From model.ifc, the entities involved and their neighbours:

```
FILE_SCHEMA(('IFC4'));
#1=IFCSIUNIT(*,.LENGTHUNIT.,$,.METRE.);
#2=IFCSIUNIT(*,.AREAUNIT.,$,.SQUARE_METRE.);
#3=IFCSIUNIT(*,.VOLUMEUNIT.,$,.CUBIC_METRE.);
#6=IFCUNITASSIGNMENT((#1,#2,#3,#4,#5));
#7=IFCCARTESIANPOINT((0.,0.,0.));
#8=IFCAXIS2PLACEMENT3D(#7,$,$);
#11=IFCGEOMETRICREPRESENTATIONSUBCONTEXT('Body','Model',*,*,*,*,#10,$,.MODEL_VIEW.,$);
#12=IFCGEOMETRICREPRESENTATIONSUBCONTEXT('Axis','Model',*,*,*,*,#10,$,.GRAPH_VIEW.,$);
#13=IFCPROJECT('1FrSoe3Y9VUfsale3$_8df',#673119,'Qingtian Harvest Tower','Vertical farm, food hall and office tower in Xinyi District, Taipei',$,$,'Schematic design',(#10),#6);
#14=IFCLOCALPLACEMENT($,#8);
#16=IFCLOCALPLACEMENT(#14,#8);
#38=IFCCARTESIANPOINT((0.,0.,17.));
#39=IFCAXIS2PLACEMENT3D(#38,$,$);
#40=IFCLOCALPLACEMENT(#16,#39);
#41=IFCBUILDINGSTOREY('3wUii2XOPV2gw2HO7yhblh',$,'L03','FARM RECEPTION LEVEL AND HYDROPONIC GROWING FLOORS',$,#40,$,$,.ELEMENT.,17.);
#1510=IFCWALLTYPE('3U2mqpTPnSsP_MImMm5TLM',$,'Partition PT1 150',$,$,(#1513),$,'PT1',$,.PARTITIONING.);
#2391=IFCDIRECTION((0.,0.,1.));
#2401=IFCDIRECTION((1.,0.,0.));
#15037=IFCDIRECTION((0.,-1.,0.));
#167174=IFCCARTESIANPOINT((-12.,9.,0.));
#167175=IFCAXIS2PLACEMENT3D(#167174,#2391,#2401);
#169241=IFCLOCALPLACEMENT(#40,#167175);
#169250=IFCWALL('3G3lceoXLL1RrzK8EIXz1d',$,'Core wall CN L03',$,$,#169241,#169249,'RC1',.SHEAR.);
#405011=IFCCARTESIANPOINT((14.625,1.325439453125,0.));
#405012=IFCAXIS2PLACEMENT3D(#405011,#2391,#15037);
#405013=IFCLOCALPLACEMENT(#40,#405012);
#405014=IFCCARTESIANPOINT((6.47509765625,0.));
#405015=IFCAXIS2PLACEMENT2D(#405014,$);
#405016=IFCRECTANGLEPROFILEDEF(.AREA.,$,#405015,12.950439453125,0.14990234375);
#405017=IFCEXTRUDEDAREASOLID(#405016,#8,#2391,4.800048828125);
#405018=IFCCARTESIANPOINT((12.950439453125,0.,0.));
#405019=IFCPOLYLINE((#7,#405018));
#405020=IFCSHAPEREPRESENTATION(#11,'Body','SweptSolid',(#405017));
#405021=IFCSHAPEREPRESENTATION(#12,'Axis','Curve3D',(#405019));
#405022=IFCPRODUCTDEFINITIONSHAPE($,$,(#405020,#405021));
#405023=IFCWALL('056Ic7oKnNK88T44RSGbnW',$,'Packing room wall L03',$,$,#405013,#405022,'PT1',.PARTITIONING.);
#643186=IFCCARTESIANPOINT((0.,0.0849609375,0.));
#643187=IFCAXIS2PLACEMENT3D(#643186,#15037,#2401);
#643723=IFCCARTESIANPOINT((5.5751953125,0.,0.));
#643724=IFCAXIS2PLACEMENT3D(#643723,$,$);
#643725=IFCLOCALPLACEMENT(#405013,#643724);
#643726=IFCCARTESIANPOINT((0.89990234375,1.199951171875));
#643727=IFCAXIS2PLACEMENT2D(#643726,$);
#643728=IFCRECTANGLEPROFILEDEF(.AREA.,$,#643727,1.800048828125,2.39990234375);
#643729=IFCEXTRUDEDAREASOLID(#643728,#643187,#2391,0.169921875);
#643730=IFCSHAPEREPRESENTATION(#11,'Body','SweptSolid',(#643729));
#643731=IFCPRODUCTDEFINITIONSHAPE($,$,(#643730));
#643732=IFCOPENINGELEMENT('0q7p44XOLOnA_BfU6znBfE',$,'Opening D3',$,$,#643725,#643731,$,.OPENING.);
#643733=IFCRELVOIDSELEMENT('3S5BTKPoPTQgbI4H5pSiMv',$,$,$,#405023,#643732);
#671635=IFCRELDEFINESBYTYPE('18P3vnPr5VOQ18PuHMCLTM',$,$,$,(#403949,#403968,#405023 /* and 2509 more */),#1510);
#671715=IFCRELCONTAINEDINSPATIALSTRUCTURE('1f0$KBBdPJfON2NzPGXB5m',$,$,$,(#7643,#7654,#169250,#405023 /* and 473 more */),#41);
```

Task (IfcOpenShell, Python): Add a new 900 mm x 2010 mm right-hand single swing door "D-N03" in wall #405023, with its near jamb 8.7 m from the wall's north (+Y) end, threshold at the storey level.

```python
import numpy as np
import ifcopenshell
import ifcopenshell.api.feature
import ifcopenshell.api.geometry
import ifcopenshell.api.root
import ifcopenshell.api.spatial
import ifcopenshell.geom
import ifcopenshell.util.element
import ifcopenshell.util.placement
import ifcopenshell.util.representation
import ifcopenshell.util.shape
import ifcopenshell.util.unit

model = ifcopenshell.open("model.ifc")
unit_scale = ifcopenshell.util.unit.calculate_unit_scale(model)
settings = ifcopenshell.geom.settings()


def volume(element):
    """Net volume in cubic metres, openings subtracted."""
    shape = ifcopenshell.geom.create_shape(settings, element)
    return ifcopenshell.util.shape.get_volume(shape.geometry)


wall = model.by_id(405023)
storey = ifcopenshell.util.element.get_container(wall, ifc_class="IfcBuildingStorey")
context = ifcopenshell.util.representation.get_context(model, "Model", "Body", "MODEL_VIEW")
before = volume(wall)

width, height, from_end, sill = 0.9, 2.01, 8.7, 0.0  # metres

# The wall runs along its own X axis, and the end named is its -X end.
wall_shape = ifcopenshell.geom.create_shape(settings, wall)
x, y, z = ifcopenshell.util.shape.get_vertices(wall_shape.geometry).T
start = x.min() + from_end
face, thickness = float(y.min()), float(y.max() - y.min())
wall_matrix = ifcopenshell.util.placement.get_local_placement(wall.ObjectPlacement)
level = ifcopenshell.util.placement.get_local_placement(storey.ObjectPlacement)[2, 3]


def in_wall(x, y):
    """Placement at x, y metres in the wall's axes, at sill height."""
    matrix = wall_matrix.copy()
    matrix[:, 3] = wall_matrix @ np.array([x / unit_scale, y / unit_scale, 0.0, 1.0])
    matrix[2, 3] = level + sill / unit_scale
    return matrix


# Opening: a box that overshoots both wall faces by 50 mm.
opening = ifcopenshell.api.root.create_entity(model, ifc_class="IfcOpeningElement", predefined_type="OPENING")
box = ifcopenshell.api.geometry.add_wall_representation(
    model, context=context, length=width, height=height, thickness=thickness + 0.1
)
ifcopenshell.api.geometry.assign_representation(model, product=opening, representation=box)
ifcopenshell.api.geometry.edit_object_placement(model, product=opening, matrix=in_wall(start, face - 0.05), is_si=False)
ifcopenshell.api.feature.add_feature(model, feature=opening, element=wall)

door = ifcopenshell.api.root.create_entity(model, ifc_class="IfcDoor", name="D-N03", predefined_type="DOOR")
door.OverallWidth, door.OverallHeight = width / unit_scale, height / unit_scale
door.OperationType = "SINGLE_SWING_RIGHT"
body = ifcopenshell.api.geometry.add_door_representation(
    model,
    context=context,
    overall_width=door.OverallWidth,
    overall_height=door.OverallHeight,
    operation_type="SINGLE_SWING_RIGHT",
    lining_properties={"LiningDepth": thickness / unit_scale, "ThresholdDepth": thickness / unit_scale},
)
ifcopenshell.api.geometry.assign_representation(model, product=door, representation=body)
ifcopenshell.api.spatial.assign_container(model, products=[door], relating_structure=storey)
ifcopenshell.api.feature.add_filling(model, opening=opening, element=door)

# The lining spans the wall, so the door starts at the wall face.
ifcopenshell.api.geometry.edit_object_placement(model, product=door, matrix=in_wall(start, face), is_si=False)

after = volume(wall)

print(f"wall volume {before:.3f} -> {after:.3f} m3")

model.write("model_edited.ifc")
```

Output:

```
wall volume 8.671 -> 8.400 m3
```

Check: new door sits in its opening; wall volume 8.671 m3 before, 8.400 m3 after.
